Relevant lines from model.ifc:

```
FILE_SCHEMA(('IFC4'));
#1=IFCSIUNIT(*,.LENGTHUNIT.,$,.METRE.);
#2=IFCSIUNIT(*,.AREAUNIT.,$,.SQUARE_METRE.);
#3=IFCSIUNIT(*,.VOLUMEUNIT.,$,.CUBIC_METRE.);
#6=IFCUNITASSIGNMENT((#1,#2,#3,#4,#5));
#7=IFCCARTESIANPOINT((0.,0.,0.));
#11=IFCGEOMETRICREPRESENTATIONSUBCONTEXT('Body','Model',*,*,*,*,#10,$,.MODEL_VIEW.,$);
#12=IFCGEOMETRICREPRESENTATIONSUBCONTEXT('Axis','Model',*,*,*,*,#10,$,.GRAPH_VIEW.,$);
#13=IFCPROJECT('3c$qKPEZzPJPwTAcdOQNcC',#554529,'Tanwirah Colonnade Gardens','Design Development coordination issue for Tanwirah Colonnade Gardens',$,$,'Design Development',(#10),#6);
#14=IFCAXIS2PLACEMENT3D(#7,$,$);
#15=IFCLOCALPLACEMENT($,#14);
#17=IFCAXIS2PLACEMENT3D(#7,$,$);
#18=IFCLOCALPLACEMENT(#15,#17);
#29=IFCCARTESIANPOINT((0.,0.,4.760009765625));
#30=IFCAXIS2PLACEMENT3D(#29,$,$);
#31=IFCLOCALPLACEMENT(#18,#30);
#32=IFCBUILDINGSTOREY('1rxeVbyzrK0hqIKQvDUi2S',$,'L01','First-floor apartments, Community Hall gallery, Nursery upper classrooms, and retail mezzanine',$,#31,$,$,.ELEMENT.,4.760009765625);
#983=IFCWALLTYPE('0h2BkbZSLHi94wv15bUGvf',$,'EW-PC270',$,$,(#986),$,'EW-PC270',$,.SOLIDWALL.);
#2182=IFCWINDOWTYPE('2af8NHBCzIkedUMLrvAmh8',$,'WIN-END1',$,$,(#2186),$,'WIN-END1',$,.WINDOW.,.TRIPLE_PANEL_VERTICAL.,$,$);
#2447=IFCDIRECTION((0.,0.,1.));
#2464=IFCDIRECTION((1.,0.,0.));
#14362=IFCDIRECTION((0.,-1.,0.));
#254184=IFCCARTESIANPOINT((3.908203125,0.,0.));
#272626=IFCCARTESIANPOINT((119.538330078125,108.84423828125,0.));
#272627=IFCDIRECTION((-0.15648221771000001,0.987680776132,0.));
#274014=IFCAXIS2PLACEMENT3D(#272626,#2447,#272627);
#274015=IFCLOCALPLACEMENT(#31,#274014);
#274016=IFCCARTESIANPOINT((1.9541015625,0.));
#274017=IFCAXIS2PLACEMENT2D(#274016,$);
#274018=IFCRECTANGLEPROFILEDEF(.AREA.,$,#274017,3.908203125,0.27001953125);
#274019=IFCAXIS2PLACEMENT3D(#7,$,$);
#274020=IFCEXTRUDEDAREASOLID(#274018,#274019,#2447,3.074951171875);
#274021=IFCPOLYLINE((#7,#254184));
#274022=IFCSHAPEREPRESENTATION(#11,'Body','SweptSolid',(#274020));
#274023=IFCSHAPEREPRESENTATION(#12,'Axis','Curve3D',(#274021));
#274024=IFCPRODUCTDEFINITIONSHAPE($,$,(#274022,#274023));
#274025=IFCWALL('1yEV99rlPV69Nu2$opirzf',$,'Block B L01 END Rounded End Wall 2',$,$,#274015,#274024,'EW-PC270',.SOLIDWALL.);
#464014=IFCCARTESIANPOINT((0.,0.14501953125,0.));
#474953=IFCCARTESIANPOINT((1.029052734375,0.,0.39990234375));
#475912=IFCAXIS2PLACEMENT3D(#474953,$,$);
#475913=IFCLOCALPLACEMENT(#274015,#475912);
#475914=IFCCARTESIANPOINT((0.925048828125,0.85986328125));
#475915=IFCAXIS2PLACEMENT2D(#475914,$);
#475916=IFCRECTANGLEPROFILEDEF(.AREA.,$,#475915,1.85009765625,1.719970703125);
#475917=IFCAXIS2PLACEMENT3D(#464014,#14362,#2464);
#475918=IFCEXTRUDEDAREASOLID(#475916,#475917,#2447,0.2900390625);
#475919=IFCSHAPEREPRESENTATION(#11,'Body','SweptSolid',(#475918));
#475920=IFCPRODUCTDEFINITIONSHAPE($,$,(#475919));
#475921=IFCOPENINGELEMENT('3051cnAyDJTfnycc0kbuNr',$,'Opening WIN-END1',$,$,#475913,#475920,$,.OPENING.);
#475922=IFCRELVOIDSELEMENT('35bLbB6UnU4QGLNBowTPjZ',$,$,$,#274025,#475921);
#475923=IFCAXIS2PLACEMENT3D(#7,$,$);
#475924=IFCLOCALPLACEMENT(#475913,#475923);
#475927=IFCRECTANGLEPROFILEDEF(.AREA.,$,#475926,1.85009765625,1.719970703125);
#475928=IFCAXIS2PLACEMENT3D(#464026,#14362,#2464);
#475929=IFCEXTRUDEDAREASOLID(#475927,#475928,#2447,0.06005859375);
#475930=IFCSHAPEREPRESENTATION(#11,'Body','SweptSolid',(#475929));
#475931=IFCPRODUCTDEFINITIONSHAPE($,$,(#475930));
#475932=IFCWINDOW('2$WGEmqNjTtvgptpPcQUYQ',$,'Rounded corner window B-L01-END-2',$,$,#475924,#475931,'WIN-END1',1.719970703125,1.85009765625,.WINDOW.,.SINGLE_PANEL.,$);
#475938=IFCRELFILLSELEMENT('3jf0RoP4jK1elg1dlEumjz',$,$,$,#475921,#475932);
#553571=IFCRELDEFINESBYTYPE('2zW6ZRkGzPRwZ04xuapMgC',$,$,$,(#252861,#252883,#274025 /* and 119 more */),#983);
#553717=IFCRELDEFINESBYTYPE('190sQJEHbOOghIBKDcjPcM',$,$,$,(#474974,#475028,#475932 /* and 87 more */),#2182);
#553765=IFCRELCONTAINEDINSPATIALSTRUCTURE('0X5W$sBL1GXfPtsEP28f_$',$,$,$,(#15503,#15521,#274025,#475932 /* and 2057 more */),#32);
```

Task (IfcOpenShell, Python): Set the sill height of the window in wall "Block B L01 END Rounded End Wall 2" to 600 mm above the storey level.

```python
import numpy as np
import ifcopenshell
import ifcopenshell.api.geometry
import ifcopenshell.geom
import ifcopenshell.util.element
import ifcopenshell.util.placement
import ifcopenshell.util.shape
import ifcopenshell.util.unit

model = ifcopenshell.open("model.ifc")
unit_scale = ifcopenshell.util.unit.calculate_unit_scale(model)

window = model.by_guid("2$WGEmqNjTtvgptpPcQUYQ")
opening = window.FillsVoids[0].RelatingOpeningElement
storey = ifcopenshell.util.element.get_container(window, ifc_class="IfcBuildingStorey")
level = ifcopenshell.util.placement.get_local_placement(storey.ObjectPlacement)[2, 3]

# The opening's origin need not be at the sill, so measure its lowest point.
shape = ifcopenshell.geom.create_shape(ifcopenshell.geom.settings(), opening)
bottom = ifcopenshell.util.shape.get_shape_bottom_elevation(shape, shape.geometry) / unit_scale
dz = level + 0.6 - bottom

shift = np.array([0.0, 0.0, dz])
# The window is placed relative to its opening, so it follows when the opening moves.
matrix = ifcopenshell.util.placement.get_local_placement(opening.ObjectPlacement)
matrix[:3, 3] += shift
ifcopenshell.api.geometry.edit_object_placement(
    model, product=opening, matrix=matrix, is_si=False, should_transform_children=True
)

print(f"moved by {dz * unit_scale:+.3f} m")

model.write("model_v2.ifc")
```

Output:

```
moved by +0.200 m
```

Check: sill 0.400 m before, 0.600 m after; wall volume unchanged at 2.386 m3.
